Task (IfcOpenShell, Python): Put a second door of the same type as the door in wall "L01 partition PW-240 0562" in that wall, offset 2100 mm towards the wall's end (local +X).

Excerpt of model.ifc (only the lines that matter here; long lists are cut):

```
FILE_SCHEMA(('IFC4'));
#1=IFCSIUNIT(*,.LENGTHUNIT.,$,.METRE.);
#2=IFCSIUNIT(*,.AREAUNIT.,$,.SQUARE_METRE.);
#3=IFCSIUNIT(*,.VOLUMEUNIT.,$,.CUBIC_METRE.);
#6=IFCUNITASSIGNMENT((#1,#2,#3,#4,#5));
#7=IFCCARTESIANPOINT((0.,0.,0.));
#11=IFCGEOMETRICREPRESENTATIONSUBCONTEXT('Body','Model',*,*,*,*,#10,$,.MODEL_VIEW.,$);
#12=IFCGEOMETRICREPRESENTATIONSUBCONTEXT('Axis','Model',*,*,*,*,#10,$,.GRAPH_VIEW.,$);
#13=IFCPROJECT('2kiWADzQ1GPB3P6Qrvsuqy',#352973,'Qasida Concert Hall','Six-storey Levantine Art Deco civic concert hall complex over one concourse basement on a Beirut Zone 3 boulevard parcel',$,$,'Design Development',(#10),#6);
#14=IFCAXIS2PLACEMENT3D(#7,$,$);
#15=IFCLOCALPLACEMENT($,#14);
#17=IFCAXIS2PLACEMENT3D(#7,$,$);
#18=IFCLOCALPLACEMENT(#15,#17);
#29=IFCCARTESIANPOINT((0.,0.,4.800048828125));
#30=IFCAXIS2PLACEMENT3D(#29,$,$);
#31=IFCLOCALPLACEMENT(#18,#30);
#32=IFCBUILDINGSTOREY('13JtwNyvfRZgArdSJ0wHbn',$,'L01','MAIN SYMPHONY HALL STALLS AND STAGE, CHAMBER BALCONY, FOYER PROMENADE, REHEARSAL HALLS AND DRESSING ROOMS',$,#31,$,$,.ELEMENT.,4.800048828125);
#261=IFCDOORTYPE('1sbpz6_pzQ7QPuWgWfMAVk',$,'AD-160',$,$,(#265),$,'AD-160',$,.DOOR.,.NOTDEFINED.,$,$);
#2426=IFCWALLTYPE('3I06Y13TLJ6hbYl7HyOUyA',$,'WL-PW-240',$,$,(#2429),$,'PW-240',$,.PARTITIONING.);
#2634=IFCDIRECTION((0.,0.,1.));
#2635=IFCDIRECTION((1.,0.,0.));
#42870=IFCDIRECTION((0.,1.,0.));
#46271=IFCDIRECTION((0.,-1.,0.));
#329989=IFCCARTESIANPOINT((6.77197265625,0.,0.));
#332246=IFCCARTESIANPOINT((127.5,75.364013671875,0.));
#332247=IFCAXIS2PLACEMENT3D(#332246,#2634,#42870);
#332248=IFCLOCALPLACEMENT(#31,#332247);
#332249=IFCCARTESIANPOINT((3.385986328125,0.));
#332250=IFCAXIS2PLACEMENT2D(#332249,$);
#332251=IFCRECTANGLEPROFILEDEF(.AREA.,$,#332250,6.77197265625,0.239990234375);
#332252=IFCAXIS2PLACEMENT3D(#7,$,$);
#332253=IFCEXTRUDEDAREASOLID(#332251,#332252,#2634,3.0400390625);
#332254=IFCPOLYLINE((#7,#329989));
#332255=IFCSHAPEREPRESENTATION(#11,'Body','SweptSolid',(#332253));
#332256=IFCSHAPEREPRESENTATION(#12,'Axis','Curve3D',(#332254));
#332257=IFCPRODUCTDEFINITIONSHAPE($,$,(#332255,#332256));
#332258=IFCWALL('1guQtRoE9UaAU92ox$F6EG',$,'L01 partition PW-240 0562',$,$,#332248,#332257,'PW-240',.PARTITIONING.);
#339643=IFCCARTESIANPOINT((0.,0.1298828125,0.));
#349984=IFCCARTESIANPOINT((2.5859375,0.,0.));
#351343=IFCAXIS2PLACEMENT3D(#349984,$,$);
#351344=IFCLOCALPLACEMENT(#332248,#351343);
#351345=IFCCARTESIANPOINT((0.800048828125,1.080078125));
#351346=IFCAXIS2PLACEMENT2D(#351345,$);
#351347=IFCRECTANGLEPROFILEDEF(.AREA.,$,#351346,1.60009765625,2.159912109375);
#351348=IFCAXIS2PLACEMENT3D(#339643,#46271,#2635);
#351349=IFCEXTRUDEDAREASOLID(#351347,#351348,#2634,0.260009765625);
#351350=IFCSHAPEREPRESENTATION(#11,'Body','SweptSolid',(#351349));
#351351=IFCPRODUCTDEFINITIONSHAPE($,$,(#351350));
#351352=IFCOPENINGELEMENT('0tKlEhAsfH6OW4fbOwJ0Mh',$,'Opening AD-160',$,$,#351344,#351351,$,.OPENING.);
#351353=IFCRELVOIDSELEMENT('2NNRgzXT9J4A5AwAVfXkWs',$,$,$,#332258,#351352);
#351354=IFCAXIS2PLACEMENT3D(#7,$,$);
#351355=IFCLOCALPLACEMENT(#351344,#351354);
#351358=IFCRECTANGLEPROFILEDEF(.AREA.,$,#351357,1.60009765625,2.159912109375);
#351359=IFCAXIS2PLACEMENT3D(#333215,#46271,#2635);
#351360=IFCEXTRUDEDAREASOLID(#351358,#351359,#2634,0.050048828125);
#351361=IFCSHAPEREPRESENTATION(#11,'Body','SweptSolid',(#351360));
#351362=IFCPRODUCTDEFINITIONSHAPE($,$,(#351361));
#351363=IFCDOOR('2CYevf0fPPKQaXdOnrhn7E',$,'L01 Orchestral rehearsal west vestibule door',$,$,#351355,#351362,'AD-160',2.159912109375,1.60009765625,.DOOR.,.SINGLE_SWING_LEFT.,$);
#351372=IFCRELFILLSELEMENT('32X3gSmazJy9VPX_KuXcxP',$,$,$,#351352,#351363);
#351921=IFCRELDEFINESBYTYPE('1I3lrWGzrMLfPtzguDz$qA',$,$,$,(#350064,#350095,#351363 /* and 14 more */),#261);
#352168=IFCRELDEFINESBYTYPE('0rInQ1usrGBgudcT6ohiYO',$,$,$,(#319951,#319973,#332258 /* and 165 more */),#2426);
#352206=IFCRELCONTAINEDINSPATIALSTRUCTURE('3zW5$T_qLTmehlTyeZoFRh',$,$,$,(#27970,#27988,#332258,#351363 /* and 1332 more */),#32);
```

```python
import ifcopenshell
import ifcopenshell.api.feature
import ifcopenshell.api.geometry
import ifcopenshell.api.root
import ifcopenshell.geom
import ifcopenshell.util.element
import ifcopenshell.util.placement
import ifcopenshell.util.shape

model = ifcopenshell.open("model.ifc")
settings = ifcopenshell.geom.settings()


def volume(element):
    """Net volume in cubic metres, openings subtracted."""
    shape = ifcopenshell.geom.create_shape(settings, element)
    return ifcopenshell.util.shape.get_volume(shape.geometry)


door = model.by_guid("2CYevf0fPPKQaXdOnrhn7E")
opening = door.FillsVoids[0].RelatingOpeningElement
wall = opening.VoidsElements[0].RelatingBuildingElement
before = volume(wall)
shift = ifcopenshell.util.placement.get_local_placement(wall.ObjectPlacement)[:3, 0] * 2.1

# copy_class copies the void relationship, type, container and properties, but no geometry.
new_opening = ifcopenshell.api.root.copy_class(model, product=opening)
new_opening.Representation = ifcopenshell.util.element.copy_deep(
    model, opening.Representation, exclude=["IfcGeometricRepresentationContext", "IfcRepresentationMap"]
)
new_door = ifcopenshell.api.root.copy_class(model, product=door)
new_door.Representation = ifcopenshell.util.element.copy_deep(
    model, door.Representation, exclude=["IfcGeometricRepresentationContext", "IfcRepresentationMap"]
)
new_door.Tag = None
ifcopenshell.api.feature.add_filling(model, opening=new_opening, element=new_door)

for old, new in ((opening, new_opening), (door, new_door)):
    matrix = ifcopenshell.util.placement.get_local_placement(old.ObjectPlacement)
    matrix[:3, 3] += shift
    ifcopenshell.api.geometry.edit_object_placement(model, product=new, matrix=matrix, is_si=False)

after = volume(wall)

print(f"wall volume {before:.3f} -> {after:.3f} m3")

model.write("model-out.ifc")
```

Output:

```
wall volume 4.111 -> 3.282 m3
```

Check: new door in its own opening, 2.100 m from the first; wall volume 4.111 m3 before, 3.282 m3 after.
